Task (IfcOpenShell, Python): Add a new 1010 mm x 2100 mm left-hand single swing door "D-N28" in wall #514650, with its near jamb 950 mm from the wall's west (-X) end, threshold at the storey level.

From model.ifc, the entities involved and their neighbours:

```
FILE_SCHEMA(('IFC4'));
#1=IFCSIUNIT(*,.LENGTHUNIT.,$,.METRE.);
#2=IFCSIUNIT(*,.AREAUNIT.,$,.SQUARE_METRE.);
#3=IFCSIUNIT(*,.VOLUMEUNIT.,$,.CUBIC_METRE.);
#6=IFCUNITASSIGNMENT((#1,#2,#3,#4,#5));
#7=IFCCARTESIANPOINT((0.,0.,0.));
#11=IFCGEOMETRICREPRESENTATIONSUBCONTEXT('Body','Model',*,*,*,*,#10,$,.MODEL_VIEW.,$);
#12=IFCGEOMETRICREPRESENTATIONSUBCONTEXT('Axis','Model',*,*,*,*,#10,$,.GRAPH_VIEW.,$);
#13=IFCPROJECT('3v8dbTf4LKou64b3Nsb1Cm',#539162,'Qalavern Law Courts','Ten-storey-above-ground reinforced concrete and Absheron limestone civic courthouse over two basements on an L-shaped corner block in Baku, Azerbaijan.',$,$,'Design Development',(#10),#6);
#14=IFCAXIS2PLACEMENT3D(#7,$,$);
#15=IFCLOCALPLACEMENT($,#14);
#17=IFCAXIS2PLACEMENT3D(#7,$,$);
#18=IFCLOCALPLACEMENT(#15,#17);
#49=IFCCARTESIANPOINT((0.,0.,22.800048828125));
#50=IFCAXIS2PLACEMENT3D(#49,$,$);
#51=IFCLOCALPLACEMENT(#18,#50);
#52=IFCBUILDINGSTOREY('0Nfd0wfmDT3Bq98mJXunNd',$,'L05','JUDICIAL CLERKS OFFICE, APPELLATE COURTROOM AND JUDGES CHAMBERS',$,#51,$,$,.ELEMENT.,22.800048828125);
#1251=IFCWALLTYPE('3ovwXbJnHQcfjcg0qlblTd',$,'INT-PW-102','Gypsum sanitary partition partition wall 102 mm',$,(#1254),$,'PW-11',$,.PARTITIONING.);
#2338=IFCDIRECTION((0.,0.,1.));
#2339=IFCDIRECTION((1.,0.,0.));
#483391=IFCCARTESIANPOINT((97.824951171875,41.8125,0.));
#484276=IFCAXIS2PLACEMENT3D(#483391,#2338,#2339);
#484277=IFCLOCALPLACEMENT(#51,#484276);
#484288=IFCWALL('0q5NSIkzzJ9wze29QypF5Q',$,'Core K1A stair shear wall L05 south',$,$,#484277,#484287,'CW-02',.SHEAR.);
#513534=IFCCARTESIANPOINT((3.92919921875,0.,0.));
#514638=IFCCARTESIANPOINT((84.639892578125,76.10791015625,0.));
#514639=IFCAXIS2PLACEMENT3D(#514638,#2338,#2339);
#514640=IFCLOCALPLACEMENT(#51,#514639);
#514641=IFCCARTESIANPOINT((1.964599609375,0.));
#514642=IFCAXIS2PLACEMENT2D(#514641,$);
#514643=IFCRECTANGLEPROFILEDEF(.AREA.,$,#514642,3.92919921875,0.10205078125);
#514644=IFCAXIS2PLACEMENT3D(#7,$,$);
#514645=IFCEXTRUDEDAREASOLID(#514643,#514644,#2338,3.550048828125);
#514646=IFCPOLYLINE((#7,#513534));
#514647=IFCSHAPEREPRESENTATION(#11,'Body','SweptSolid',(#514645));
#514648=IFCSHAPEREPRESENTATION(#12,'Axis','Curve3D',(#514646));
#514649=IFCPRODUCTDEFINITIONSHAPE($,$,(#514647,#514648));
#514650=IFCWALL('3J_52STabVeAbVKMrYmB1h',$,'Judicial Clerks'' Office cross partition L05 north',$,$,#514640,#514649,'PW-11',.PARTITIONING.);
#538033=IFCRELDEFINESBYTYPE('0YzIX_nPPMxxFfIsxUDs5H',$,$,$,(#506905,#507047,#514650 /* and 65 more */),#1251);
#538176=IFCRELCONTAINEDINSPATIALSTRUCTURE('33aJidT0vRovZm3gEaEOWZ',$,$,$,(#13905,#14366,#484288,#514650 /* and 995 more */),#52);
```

```python
import numpy as np
import ifcopenshell
import ifcopenshell.api.feature
import ifcopenshell.api.geometry
import ifcopenshell.api.root
import ifcopenshell.api.spatial
import ifcopenshell.geom
import ifcopenshell.util.element
import ifcopenshell.util.placement
import ifcopenshell.util.representation
import ifcopenshell.util.shape
import ifcopenshell.util.unit

model = ifcopenshell.open("model.ifc")
unit_scale = ifcopenshell.util.unit.calculate_unit_scale(model)
settings = ifcopenshell.geom.settings()


def volume(element):
    """Net volume in cubic metres, openings subtracted."""
    shape = ifcopenshell.geom.create_shape(settings, element)
    return ifcopenshell.util.shape.get_volume(shape.geometry)


wall = model.by_id(514650)
storey = ifcopenshell.util.element.get_container(wall, ifc_class="IfcBuildingStorey")
context = ifcopenshell.util.representation.get_context(model, "Model", "Body", "MODEL_VIEW")
before = volume(wall)

width, height, from_end, sill = 1.01, 2.1, 0.95, 0.0  # metres

# The wall runs along its own X axis, and the end named is its -X end.
wall_shape = ifcopenshell.geom.create_shape(settings, wall)
x, y, z = ifcopenshell.util.shape.get_vertices(wall_shape.geometry).T
start = x.min() + from_end
face, thickness = float(y.min()), float(y.max() - y.min())
wall_matrix = ifcopenshell.util.placement.get_local_placement(wall.ObjectPlacement)
level = ifcopenshell.util.placement.get_local_placement(storey.ObjectPlacement)[2, 3]


def in_wall(x, y):
    """Placement at x, y metres in the wall's axes, at sill height."""
    matrix = wall_matrix.copy()
    matrix[:, 3] = wall_matrix @ np.array([x / unit_scale, y / unit_scale, 0.0, 1.0])
    matrix[2, 3] = level + sill / unit_scale
    return matrix


# Opening: a box that overshoots both wall faces by 50 mm.
opening = ifcopenshell.api.root.create_entity(model, ifc_class="IfcOpeningElement", predefined_type="OPENING")
box = ifcopenshell.api.geometry.add_wall_representation(
    model, context=context, length=width, height=height, thickness=thickness + 0.1
)
ifcopenshell.api.geometry.assign_representation(model, product=opening, representation=box)
ifcopenshell.api.geometry.edit_object_placement(model, product=opening, matrix=in_wall(start, face - 0.05), is_si=False)
ifcopenshell.api.feature.add_feature(model, feature=opening, element=wall)

door = ifcopenshell.api.root.create_entity(model, ifc_class="IfcDoor", name="D-N28", predefined_type="DOOR")
door.OverallWidth, door.OverallHeight = width / unit_scale, height / unit_scale
door.OperationType = "SINGLE_SWING_LEFT"
body = ifcopenshell.api.geometry.add_door_representation(
    model,
    context=context,
    overall_width=door.OverallWidth,
    overall_height=door.OverallHeight,
    operation_type="SINGLE_SWING_LEFT",
    lining_properties={"LiningDepth": thickness / unit_scale, "ThresholdDepth": thickness / unit_scale},
)
ifcopenshell.api.geometry.assign_representation(model, product=door, representation=body)
ifcopenshell.api.spatial.assign_container(model, products=[door], relating_structure=storey)
ifcopenshell.api.feature.add_filling(model, opening=opening, element=door)

# The lining spans the wall, so the door starts at the wall face.
ifcopenshell.api.geometry.edit_object_placement(model, product=door, matrix=in_wall(start, face), is_si=False)

after = volume(wall)

print(f"wall volume {before:.3f} -> {after:.3f} m3")

model.write("model_edited.ifc")
```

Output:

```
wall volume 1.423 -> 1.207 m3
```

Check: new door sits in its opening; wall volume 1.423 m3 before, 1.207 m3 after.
